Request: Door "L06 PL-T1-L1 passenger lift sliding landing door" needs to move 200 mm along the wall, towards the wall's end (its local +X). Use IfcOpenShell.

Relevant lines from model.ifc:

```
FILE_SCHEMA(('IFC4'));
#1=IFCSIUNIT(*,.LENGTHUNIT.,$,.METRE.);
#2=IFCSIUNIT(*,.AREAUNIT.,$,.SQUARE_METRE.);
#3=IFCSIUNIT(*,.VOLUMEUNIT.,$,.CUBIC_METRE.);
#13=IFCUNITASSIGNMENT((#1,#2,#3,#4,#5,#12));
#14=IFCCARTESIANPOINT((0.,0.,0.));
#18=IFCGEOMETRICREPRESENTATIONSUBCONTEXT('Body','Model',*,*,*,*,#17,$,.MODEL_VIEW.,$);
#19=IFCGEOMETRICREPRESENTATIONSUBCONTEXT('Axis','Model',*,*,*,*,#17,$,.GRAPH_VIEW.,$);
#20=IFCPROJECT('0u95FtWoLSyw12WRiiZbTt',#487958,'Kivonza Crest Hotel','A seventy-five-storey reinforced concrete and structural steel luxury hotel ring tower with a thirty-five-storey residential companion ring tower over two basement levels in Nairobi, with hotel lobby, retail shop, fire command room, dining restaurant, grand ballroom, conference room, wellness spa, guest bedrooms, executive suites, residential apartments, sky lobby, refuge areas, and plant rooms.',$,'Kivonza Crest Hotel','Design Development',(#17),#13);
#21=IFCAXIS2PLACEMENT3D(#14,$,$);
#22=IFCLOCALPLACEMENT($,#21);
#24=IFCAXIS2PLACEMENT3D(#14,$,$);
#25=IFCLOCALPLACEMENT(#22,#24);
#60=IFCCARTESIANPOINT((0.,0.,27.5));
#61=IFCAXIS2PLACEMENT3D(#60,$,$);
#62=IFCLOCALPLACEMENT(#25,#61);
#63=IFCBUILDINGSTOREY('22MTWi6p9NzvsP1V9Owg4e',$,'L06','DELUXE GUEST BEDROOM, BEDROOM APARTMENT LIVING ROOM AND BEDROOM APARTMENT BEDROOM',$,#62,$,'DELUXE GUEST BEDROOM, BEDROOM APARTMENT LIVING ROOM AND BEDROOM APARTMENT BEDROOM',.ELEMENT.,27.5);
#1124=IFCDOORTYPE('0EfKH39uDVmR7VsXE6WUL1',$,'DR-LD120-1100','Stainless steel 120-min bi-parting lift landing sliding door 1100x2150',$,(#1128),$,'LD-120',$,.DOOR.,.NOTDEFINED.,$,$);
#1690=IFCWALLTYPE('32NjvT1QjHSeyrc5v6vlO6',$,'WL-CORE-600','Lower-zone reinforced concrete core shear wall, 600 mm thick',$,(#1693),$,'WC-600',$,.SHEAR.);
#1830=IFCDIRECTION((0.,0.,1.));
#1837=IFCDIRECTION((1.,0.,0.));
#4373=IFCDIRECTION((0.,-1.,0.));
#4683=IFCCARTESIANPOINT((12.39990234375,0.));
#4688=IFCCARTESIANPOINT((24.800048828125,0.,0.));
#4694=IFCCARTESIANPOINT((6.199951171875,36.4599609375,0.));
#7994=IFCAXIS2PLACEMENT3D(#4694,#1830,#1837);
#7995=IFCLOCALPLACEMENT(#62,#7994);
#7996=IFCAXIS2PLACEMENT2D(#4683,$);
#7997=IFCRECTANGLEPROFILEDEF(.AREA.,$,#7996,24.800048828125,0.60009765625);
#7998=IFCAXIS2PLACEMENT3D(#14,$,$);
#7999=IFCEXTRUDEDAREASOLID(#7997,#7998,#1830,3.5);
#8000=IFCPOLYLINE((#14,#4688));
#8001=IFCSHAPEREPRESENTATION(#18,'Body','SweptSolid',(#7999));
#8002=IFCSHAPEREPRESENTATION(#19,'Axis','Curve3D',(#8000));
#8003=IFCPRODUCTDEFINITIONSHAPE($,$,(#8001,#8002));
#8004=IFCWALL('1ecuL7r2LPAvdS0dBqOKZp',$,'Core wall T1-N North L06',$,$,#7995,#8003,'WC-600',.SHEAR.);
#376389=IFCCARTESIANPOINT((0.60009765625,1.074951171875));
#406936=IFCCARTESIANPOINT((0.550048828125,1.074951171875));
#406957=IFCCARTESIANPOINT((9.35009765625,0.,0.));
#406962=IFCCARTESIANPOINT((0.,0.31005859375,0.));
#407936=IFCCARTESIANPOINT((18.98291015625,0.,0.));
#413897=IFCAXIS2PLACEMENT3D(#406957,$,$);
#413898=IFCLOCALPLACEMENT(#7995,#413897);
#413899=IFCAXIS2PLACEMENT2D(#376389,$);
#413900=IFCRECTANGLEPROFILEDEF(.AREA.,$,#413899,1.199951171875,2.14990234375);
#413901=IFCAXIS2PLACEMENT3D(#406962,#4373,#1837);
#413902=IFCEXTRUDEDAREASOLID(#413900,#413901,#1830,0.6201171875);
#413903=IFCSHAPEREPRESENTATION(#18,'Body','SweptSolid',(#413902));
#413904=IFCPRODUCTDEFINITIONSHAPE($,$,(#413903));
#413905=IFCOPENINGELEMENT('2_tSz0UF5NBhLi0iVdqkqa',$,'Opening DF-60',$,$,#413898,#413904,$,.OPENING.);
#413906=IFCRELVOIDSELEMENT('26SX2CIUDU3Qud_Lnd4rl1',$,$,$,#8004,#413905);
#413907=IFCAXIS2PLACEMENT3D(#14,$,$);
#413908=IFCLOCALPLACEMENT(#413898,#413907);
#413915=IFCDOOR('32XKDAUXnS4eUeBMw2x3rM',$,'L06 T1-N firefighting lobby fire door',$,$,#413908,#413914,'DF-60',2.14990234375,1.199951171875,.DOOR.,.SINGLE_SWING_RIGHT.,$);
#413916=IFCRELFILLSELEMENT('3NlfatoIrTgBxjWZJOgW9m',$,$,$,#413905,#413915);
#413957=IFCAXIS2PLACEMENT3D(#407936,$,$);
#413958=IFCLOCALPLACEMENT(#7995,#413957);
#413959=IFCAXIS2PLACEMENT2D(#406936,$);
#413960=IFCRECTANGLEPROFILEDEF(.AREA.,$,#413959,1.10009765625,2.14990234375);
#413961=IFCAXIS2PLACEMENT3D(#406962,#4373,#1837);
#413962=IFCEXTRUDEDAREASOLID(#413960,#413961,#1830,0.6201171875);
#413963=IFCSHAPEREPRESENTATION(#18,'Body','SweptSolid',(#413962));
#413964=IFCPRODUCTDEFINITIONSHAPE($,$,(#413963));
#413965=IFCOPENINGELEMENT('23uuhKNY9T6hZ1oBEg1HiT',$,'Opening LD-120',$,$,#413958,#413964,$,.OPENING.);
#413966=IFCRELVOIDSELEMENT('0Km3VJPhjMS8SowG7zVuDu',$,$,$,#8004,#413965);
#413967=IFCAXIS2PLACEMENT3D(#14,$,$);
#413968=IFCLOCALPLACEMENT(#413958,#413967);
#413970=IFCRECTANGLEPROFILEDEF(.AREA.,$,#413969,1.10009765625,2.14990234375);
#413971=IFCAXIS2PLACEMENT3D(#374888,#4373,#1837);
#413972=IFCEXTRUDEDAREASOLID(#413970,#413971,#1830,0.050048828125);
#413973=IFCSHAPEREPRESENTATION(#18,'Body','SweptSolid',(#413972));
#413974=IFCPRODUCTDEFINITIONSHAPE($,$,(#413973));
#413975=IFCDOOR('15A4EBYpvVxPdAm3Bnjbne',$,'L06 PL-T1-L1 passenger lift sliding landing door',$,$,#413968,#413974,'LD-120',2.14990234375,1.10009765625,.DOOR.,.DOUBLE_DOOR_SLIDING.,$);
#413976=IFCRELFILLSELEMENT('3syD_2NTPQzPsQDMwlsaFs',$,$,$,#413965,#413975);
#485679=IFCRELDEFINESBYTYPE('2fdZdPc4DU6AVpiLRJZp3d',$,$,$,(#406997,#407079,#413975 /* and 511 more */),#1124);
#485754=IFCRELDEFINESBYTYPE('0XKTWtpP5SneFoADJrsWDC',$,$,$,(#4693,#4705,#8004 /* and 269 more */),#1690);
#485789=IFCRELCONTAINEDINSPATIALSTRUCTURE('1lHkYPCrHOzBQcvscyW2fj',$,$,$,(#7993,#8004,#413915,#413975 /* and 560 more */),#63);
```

```python
import ifcopenshell
import ifcopenshell.api.geometry
import ifcopenshell.util.placement

model = ifcopenshell.open("model.ifc")

door = model.by_guid("15A4EBYpvVxPdAm3Bnjbne")
opening = door.FillsVoids[0].RelatingOpeningElement
wall = opening.VoidsElements[0].RelatingBuildingElement

wall_matrix = ifcopenshell.util.placement.get_local_placement(wall.ObjectPlacement)
shift = wall_matrix[:3, 0] * 0.2
before = ifcopenshell.util.placement.get_local_placement(door.ObjectPlacement)[:3, 3].copy()

# The door is placed relative to its opening, so it follows when the opening moves.
matrix = ifcopenshell.util.placement.get_local_placement(opening.ObjectPlacement)
matrix[:3, 3] += shift
ifcopenshell.api.geometry.edit_object_placement(
    model, product=opening, matrix=matrix, is_si=False, should_transform_children=True
)

after = ifcopenshell.util.placement.get_local_placement(door.ObjectPlacement)[:3, 3]
print("door moved by", (after - before).round(3) + 0.0)

model.write("model-out.ifc")
```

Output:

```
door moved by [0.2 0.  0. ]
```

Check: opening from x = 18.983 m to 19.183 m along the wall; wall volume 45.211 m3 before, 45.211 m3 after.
